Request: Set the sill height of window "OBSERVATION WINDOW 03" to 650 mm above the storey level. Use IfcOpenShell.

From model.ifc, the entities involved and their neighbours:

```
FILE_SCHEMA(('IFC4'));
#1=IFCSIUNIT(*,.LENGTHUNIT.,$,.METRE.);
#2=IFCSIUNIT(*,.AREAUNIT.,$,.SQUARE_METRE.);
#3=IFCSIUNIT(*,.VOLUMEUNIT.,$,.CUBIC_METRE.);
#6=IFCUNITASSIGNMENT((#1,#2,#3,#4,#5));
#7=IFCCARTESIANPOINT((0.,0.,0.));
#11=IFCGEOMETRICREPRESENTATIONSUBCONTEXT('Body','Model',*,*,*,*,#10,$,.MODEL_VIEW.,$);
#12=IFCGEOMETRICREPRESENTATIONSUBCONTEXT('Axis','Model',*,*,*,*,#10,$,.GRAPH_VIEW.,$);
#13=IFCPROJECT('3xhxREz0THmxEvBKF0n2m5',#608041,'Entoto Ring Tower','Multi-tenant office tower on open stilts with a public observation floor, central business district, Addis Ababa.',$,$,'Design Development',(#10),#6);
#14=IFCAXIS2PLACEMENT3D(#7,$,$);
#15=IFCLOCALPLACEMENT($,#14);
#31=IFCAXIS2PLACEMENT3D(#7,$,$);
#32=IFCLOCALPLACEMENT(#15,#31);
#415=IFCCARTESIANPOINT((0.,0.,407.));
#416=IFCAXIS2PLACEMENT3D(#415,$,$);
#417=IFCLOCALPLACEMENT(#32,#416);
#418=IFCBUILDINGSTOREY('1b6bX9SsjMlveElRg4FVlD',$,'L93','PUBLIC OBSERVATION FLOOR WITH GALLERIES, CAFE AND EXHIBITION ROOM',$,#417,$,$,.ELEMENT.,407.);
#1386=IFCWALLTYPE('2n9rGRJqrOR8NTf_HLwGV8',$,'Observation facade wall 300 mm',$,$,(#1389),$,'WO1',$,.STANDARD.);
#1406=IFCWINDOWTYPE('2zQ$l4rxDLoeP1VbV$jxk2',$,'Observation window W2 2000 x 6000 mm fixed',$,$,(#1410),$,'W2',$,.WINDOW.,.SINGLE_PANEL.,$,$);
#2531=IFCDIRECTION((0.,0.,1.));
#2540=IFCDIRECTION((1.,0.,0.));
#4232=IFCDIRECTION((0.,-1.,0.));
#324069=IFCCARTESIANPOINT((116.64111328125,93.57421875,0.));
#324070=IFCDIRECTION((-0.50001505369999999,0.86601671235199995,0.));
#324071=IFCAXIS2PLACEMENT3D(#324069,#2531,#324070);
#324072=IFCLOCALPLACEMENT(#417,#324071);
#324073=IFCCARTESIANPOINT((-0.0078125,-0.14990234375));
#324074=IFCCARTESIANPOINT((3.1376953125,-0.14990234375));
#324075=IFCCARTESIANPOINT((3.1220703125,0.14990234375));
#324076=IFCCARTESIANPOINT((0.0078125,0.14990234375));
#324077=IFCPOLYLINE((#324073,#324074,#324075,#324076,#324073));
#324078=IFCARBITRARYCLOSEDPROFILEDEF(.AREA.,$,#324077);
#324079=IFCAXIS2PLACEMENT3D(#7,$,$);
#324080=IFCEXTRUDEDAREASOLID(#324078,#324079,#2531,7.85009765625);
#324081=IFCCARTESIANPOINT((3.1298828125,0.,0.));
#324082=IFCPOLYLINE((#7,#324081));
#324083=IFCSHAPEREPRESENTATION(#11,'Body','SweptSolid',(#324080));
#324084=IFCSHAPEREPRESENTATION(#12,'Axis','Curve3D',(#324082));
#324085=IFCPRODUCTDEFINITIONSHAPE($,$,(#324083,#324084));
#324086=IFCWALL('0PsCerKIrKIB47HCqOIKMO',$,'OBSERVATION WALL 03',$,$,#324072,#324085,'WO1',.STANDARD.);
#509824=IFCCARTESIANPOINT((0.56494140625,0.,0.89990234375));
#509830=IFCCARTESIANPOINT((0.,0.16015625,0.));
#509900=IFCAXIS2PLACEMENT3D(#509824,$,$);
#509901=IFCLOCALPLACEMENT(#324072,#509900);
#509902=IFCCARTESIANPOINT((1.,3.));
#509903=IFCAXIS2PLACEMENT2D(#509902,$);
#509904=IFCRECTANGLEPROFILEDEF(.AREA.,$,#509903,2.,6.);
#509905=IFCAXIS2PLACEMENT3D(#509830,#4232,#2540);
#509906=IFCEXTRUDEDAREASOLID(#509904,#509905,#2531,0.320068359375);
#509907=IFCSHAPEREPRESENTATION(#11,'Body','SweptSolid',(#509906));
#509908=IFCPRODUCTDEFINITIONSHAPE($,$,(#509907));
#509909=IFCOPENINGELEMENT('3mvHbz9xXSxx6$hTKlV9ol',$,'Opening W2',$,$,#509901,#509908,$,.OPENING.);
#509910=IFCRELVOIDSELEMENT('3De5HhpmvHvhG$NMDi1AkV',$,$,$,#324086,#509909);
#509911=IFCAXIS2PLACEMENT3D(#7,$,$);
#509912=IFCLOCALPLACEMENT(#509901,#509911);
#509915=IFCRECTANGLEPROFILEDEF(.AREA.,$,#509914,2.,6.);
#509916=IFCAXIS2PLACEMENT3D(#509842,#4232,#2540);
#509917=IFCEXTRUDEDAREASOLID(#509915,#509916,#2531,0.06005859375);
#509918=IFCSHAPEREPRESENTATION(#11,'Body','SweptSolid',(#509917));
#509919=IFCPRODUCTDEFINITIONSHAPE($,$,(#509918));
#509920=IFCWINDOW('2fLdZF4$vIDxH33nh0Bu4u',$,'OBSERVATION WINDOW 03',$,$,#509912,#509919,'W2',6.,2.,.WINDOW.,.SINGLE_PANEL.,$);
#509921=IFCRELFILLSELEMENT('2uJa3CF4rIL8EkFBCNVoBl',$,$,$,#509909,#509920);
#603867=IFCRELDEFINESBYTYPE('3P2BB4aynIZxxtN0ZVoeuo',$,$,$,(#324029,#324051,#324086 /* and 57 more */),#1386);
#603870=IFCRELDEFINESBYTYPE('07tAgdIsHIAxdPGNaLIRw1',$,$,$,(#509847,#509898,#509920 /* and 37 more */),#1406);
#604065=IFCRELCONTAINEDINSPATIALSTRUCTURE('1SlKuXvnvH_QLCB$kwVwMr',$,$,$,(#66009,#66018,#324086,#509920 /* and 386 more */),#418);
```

```python
import numpy as np
import ifcopenshell
import ifcopenshell.api.geometry
import ifcopenshell.geom
import ifcopenshell.util.element
import ifcopenshell.util.placement
import ifcopenshell.util.shape
import ifcopenshell.util.unit

model = ifcopenshell.open("model.ifc")
unit_scale = ifcopenshell.util.unit.calculate_unit_scale(model)

window = model.by_id(509920)
opening = window.FillsVoids[0].RelatingOpeningElement
storey = ifcopenshell.util.element.get_container(window, ifc_class="IfcBuildingStorey")
level = ifcopenshell.util.placement.get_local_placement(storey.ObjectPlacement)[2, 3]

# The opening's origin need not be at the sill, so measure its lowest point.
shape = ifcopenshell.geom.create_shape(ifcopenshell.geom.settings(), opening)
bottom = ifcopenshell.util.shape.get_shape_bottom_elevation(shape, shape.geometry) / unit_scale
dz = level + 0.65 / unit_scale - bottom

shift = np.array([0.0, 0.0, dz])
# The window is placed relative to its opening, so it follows when the opening moves.
matrix = ifcopenshell.util.placement.get_local_placement(opening.ObjectPlacement)
matrix[:3, 3] += shift
ifcopenshell.api.geometry.edit_object_placement(
    model, product=opening, matrix=matrix, is_si=False, should_transform_children=True
)

print(f"moved by {dz * unit_scale:+.3f} m")

model.write("model_edited.ifc")
```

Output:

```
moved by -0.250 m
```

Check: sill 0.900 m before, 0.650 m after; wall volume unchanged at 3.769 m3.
